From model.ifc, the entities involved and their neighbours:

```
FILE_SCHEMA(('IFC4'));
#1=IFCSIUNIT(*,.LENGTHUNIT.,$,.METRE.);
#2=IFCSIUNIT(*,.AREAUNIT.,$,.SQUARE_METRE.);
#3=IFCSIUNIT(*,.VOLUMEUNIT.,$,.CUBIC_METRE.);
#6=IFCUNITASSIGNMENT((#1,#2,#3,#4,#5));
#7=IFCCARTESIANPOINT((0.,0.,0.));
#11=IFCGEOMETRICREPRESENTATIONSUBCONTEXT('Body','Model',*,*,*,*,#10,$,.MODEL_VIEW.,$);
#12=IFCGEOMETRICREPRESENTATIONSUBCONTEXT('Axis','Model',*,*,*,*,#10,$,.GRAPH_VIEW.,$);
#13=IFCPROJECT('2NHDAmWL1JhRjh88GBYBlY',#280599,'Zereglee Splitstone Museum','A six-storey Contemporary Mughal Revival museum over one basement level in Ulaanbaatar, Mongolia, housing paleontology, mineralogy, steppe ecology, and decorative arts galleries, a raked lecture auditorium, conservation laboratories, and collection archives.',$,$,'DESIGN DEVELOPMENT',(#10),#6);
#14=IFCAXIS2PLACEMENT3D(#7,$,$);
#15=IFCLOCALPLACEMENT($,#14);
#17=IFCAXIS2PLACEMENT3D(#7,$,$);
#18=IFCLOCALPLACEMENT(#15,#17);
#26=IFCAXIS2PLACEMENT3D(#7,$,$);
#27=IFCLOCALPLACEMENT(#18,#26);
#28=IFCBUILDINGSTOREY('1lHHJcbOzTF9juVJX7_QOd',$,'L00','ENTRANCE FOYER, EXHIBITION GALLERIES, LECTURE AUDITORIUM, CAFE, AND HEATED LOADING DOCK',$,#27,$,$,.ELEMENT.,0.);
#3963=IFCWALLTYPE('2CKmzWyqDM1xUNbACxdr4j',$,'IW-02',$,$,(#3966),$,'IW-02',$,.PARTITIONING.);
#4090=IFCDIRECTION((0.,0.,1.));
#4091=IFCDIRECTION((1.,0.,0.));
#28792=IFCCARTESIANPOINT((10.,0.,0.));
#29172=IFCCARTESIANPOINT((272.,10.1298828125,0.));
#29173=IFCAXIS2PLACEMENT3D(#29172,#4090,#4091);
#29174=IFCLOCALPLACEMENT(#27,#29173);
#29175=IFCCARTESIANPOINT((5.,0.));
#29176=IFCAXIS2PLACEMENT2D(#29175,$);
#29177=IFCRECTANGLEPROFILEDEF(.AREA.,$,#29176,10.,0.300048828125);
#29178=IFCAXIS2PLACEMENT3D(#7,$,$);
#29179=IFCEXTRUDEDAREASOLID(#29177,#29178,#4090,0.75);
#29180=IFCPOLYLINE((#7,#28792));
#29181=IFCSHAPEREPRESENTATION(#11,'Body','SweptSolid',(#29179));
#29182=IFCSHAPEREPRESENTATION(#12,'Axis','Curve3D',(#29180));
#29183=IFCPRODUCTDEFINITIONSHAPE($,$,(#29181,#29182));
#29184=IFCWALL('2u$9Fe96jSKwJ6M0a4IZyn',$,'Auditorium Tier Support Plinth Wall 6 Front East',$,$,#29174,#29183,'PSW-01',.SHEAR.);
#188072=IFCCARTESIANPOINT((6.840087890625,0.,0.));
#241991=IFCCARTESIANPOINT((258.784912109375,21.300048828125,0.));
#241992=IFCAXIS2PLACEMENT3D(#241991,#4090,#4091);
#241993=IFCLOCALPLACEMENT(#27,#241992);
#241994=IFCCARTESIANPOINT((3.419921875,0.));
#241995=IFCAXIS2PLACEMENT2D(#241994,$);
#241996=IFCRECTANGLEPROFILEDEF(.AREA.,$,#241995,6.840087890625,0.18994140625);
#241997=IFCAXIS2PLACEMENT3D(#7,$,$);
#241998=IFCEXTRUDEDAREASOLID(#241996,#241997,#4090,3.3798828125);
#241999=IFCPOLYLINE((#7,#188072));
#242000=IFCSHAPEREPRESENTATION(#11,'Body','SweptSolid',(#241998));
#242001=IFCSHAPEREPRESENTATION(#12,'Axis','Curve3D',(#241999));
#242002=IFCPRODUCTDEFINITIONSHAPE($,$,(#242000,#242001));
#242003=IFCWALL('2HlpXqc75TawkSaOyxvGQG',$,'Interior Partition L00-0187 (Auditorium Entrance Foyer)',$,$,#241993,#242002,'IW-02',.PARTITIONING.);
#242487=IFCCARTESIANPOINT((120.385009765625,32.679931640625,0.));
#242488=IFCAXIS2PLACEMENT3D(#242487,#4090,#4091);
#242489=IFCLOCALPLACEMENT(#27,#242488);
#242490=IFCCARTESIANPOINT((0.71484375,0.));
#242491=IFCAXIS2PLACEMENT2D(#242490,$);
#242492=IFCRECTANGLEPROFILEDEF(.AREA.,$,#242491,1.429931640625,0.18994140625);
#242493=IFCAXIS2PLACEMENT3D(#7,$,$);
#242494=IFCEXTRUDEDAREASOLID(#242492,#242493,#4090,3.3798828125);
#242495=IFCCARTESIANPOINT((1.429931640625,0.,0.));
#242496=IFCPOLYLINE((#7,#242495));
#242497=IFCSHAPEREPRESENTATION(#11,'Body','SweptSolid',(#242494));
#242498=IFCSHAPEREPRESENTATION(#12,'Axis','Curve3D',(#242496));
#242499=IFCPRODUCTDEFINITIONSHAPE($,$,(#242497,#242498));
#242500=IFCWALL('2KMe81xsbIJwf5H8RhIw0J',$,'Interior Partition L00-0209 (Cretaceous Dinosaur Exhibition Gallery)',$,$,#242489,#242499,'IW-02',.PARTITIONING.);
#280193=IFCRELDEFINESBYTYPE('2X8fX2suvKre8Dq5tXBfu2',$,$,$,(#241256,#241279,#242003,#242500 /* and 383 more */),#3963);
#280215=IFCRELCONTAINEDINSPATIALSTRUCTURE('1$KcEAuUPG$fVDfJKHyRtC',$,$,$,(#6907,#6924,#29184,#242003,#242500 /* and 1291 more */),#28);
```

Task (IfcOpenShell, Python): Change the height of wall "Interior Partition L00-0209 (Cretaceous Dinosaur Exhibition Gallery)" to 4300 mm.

```python
import ifcopenshell
import ifcopenshell.geom
import ifcopenshell.util.representation
import ifcopenshell.util.shape
import ifcopenshell.util.unit

model = ifcopenshell.open("model.ifc")
unit_scale = ifcopenshell.util.unit.calculate_unit_scale(model)
settings = ifcopenshell.geom.settings()


def volume(element):
    """Net volume in cubic metres, openings subtracted."""
    shape = ifcopenshell.geom.create_shape(settings, element)
    return ifcopenshell.util.shape.get_volume(shape.geometry)


wall = model.by_guid("2KMe81xsbIJwf5H8RhIw0J")
before = volume(wall)

body = ifcopenshell.util.representation.get_representation(wall, "Model", "Body")
solid = body.Items[0]
old_height = solid.Depth
solid.Depth = 4.3 / unit_scale
after = volume(wall)

print(f"height {old_height:g} -> {solid.Depth:g}, volume {before:.3f} -> {after:.3f} m3")

model.write("model_rev.ifc")
```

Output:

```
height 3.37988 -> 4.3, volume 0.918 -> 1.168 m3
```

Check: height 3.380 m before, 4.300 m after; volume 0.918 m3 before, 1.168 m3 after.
